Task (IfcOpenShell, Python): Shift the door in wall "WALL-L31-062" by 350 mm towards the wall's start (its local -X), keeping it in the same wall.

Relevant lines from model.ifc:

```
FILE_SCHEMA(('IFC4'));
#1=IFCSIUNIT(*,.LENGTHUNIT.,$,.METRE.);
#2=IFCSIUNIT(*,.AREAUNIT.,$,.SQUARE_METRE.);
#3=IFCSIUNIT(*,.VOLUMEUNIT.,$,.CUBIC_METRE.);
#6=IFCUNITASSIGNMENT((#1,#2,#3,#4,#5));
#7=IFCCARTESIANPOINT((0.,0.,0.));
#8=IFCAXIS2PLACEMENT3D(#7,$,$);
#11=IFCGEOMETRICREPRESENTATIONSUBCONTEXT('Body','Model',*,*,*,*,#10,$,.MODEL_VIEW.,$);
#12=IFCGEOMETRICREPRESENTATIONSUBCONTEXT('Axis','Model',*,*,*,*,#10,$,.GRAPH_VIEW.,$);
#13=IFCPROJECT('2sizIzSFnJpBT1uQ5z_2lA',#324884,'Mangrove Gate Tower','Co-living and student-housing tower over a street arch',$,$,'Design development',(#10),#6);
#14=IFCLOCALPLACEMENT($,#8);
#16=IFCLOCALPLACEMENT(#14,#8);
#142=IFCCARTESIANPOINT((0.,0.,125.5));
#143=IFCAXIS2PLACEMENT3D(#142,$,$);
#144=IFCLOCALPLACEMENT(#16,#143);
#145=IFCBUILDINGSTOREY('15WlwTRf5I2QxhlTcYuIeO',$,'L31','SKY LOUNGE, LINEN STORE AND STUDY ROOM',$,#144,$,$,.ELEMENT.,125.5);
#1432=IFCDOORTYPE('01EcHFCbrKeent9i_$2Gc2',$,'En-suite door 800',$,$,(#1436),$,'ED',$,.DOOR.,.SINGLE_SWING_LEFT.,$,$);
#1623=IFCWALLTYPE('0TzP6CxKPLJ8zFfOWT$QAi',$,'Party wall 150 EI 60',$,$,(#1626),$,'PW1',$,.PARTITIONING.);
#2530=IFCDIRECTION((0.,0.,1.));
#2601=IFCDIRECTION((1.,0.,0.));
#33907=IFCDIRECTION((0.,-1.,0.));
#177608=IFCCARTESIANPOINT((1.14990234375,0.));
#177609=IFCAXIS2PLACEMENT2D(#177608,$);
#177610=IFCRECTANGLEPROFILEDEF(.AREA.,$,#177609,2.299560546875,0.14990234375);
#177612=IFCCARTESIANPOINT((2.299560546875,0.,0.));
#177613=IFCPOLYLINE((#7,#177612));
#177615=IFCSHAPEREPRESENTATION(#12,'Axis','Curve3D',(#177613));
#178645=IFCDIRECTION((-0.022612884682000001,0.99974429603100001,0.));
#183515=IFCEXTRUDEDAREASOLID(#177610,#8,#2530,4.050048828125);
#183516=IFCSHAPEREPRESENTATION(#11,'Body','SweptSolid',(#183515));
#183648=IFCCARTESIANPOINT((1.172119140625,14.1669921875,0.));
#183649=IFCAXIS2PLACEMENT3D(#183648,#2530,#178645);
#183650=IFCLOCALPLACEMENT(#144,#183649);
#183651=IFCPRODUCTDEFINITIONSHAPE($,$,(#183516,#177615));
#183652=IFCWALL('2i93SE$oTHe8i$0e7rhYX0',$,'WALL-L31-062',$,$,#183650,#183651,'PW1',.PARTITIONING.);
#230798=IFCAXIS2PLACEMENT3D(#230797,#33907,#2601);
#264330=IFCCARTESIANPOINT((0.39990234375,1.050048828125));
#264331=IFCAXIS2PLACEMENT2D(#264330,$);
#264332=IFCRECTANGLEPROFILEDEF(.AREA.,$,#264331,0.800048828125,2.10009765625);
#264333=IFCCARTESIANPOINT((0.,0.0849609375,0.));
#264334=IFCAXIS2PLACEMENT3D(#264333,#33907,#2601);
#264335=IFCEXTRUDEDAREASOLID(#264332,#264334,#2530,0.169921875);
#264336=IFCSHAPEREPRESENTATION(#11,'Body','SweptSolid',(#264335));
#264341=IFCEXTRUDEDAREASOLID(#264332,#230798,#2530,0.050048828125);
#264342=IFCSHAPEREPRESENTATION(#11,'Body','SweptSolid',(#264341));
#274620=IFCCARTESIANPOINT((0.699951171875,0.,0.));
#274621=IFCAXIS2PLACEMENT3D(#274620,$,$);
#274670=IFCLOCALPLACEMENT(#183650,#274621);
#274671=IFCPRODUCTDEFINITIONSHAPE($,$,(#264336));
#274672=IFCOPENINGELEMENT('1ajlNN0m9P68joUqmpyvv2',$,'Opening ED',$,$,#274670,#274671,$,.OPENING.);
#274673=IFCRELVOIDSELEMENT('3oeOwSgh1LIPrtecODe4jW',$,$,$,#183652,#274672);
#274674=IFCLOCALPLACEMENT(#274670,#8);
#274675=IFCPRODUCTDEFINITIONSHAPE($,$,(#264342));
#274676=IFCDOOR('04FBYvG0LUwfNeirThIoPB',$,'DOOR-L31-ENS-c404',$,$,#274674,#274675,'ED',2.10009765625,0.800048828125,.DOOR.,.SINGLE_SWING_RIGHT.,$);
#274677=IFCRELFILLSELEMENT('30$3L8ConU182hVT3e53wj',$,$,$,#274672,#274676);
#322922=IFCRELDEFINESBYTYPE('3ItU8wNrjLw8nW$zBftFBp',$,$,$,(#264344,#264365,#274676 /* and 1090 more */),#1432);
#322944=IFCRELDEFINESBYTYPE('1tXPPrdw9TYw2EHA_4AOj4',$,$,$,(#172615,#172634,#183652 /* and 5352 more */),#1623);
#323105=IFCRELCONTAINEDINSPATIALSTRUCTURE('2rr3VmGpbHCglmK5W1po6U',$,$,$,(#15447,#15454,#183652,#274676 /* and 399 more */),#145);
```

```python
import ifcopenshell
import ifcopenshell.api.geometry
import ifcopenshell.util.placement

model = ifcopenshell.open("model.ifc")

door = model.by_guid("04FBYvG0LUwfNeirThIoPB")
opening = door.FillsVoids[0].RelatingOpeningElement
wall = opening.VoidsElements[0].RelatingBuildingElement

wall_matrix = ifcopenshell.util.placement.get_local_placement(wall.ObjectPlacement)
shift = wall_matrix[:3, 0] * -0.35
before = ifcopenshell.util.placement.get_local_placement(door.ObjectPlacement)[:3, 3].copy()

# The door is placed relative to its opening, so it follows when the opening moves.
matrix = ifcopenshell.util.placement.get_local_placement(opening.ObjectPlacement)
matrix[:3, 3] += shift
ifcopenshell.api.geometry.edit_object_placement(
    model, product=opening, matrix=matrix, is_si=False, should_transform_children=True
)

after = ifcopenshell.util.placement.get_local_placement(door.ObjectPlacement)[:3, 3]
print("door moved by", (after - before).round(3) + 0.0)

model.write("model_edited.ifc")
```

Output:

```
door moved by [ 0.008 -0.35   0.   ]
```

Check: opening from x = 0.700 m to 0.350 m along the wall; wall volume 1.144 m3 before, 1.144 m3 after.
